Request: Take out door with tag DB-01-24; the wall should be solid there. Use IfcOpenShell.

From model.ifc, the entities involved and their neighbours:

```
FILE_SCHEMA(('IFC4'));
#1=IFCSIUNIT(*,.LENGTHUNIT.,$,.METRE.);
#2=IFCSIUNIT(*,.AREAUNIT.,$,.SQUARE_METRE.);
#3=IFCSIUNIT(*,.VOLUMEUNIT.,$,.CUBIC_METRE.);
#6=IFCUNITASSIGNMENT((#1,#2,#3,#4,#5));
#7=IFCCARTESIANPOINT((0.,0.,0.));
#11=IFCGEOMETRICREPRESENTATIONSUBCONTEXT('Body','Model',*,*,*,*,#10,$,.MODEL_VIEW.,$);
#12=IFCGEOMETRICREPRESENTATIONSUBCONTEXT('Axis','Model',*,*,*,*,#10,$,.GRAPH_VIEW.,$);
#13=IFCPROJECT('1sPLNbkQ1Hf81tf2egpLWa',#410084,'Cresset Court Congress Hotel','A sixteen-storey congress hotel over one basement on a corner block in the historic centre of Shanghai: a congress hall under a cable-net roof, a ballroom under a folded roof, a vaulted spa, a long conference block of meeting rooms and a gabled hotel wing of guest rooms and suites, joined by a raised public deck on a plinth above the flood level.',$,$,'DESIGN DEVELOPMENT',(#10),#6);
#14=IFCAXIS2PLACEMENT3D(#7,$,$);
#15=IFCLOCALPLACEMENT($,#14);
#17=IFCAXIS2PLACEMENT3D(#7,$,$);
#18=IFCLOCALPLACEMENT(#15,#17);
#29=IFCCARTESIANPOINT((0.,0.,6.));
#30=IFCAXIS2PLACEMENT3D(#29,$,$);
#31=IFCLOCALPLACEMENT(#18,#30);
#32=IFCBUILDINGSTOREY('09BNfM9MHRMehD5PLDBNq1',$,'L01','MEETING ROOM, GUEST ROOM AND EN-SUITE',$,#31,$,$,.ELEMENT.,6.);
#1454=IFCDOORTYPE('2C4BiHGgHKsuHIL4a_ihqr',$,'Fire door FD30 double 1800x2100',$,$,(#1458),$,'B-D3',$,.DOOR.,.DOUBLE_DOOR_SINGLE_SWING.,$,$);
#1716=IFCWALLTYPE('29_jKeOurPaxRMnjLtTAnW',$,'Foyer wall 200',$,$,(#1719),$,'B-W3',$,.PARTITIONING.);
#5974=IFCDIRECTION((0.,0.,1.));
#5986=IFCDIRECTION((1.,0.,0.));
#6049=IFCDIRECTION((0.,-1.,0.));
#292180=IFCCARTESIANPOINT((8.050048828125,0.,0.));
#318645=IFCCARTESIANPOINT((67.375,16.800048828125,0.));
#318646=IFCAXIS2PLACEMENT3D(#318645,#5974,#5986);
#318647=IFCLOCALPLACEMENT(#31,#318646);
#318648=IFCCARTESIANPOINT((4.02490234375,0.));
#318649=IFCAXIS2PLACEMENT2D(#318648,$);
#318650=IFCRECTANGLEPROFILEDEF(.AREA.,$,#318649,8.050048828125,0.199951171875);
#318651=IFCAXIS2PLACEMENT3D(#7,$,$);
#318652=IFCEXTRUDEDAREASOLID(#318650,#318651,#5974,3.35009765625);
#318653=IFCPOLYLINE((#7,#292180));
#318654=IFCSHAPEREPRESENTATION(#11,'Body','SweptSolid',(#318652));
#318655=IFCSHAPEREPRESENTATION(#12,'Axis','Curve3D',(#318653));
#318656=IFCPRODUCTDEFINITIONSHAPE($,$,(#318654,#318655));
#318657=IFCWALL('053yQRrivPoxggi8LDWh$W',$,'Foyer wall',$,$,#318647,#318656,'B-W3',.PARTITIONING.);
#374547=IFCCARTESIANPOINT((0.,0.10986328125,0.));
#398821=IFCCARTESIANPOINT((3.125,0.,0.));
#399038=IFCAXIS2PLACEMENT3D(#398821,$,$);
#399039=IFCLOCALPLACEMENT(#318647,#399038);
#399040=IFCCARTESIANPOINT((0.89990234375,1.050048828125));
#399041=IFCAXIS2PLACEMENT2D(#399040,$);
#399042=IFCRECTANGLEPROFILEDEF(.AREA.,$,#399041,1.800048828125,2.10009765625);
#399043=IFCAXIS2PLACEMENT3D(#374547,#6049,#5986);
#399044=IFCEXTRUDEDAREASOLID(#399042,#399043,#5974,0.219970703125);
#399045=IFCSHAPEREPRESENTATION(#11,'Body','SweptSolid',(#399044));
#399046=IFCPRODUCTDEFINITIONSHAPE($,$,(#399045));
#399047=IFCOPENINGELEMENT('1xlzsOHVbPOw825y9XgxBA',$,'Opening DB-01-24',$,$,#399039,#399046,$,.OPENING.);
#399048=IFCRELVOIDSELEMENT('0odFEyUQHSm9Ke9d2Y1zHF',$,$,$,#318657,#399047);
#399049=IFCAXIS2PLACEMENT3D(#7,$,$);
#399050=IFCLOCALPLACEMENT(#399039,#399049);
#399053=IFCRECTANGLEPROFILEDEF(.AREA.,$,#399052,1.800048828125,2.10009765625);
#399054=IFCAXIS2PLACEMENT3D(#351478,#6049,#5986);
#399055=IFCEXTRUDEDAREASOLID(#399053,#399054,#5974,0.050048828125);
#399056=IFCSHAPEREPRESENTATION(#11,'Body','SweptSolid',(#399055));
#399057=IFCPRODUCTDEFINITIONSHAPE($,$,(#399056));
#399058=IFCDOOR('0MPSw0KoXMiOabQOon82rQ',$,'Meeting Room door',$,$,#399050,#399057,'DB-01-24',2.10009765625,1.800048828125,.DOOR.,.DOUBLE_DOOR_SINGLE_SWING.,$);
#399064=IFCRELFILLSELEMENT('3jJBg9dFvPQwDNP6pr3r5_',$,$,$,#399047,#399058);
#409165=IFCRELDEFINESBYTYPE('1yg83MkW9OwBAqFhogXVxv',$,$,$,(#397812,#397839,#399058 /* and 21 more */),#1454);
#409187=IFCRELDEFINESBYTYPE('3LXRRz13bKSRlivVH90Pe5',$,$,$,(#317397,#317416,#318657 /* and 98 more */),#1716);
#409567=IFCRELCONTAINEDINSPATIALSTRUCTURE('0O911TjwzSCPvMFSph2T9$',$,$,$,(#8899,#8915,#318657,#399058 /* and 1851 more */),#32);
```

```python
import ifcopenshell
import ifcopenshell.api.feature
import ifcopenshell.api.root
import ifcopenshell.geom
import ifcopenshell.util.shape

model = ifcopenshell.open("model.ifc")
settings = ifcopenshell.geom.settings()


def volume(element):
    """Net volume in cubic metres, openings subtracted."""
    shape = ifcopenshell.geom.create_shape(settings, element)
    return ifcopenshell.util.shape.get_volume(shape.geometry)


door = model.by_guid("0MPSw0KoXMiOabQOon82rQ")
opening = door.FillsVoids[0].RelatingOpeningElement
wall = opening.VoidsElements[0].RelatingBuildingElement
before = volume(wall)

ifcopenshell.api.root.remove_product(model, product=door)
ifcopenshell.api.feature.remove_feature(model, feature=opening)

after = volume(wall)

print(f"wall volume {before:.3f} -> {after:.3f} m3")

model.write("model_v2.ifc")
```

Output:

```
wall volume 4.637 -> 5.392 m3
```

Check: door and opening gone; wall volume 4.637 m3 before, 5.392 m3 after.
